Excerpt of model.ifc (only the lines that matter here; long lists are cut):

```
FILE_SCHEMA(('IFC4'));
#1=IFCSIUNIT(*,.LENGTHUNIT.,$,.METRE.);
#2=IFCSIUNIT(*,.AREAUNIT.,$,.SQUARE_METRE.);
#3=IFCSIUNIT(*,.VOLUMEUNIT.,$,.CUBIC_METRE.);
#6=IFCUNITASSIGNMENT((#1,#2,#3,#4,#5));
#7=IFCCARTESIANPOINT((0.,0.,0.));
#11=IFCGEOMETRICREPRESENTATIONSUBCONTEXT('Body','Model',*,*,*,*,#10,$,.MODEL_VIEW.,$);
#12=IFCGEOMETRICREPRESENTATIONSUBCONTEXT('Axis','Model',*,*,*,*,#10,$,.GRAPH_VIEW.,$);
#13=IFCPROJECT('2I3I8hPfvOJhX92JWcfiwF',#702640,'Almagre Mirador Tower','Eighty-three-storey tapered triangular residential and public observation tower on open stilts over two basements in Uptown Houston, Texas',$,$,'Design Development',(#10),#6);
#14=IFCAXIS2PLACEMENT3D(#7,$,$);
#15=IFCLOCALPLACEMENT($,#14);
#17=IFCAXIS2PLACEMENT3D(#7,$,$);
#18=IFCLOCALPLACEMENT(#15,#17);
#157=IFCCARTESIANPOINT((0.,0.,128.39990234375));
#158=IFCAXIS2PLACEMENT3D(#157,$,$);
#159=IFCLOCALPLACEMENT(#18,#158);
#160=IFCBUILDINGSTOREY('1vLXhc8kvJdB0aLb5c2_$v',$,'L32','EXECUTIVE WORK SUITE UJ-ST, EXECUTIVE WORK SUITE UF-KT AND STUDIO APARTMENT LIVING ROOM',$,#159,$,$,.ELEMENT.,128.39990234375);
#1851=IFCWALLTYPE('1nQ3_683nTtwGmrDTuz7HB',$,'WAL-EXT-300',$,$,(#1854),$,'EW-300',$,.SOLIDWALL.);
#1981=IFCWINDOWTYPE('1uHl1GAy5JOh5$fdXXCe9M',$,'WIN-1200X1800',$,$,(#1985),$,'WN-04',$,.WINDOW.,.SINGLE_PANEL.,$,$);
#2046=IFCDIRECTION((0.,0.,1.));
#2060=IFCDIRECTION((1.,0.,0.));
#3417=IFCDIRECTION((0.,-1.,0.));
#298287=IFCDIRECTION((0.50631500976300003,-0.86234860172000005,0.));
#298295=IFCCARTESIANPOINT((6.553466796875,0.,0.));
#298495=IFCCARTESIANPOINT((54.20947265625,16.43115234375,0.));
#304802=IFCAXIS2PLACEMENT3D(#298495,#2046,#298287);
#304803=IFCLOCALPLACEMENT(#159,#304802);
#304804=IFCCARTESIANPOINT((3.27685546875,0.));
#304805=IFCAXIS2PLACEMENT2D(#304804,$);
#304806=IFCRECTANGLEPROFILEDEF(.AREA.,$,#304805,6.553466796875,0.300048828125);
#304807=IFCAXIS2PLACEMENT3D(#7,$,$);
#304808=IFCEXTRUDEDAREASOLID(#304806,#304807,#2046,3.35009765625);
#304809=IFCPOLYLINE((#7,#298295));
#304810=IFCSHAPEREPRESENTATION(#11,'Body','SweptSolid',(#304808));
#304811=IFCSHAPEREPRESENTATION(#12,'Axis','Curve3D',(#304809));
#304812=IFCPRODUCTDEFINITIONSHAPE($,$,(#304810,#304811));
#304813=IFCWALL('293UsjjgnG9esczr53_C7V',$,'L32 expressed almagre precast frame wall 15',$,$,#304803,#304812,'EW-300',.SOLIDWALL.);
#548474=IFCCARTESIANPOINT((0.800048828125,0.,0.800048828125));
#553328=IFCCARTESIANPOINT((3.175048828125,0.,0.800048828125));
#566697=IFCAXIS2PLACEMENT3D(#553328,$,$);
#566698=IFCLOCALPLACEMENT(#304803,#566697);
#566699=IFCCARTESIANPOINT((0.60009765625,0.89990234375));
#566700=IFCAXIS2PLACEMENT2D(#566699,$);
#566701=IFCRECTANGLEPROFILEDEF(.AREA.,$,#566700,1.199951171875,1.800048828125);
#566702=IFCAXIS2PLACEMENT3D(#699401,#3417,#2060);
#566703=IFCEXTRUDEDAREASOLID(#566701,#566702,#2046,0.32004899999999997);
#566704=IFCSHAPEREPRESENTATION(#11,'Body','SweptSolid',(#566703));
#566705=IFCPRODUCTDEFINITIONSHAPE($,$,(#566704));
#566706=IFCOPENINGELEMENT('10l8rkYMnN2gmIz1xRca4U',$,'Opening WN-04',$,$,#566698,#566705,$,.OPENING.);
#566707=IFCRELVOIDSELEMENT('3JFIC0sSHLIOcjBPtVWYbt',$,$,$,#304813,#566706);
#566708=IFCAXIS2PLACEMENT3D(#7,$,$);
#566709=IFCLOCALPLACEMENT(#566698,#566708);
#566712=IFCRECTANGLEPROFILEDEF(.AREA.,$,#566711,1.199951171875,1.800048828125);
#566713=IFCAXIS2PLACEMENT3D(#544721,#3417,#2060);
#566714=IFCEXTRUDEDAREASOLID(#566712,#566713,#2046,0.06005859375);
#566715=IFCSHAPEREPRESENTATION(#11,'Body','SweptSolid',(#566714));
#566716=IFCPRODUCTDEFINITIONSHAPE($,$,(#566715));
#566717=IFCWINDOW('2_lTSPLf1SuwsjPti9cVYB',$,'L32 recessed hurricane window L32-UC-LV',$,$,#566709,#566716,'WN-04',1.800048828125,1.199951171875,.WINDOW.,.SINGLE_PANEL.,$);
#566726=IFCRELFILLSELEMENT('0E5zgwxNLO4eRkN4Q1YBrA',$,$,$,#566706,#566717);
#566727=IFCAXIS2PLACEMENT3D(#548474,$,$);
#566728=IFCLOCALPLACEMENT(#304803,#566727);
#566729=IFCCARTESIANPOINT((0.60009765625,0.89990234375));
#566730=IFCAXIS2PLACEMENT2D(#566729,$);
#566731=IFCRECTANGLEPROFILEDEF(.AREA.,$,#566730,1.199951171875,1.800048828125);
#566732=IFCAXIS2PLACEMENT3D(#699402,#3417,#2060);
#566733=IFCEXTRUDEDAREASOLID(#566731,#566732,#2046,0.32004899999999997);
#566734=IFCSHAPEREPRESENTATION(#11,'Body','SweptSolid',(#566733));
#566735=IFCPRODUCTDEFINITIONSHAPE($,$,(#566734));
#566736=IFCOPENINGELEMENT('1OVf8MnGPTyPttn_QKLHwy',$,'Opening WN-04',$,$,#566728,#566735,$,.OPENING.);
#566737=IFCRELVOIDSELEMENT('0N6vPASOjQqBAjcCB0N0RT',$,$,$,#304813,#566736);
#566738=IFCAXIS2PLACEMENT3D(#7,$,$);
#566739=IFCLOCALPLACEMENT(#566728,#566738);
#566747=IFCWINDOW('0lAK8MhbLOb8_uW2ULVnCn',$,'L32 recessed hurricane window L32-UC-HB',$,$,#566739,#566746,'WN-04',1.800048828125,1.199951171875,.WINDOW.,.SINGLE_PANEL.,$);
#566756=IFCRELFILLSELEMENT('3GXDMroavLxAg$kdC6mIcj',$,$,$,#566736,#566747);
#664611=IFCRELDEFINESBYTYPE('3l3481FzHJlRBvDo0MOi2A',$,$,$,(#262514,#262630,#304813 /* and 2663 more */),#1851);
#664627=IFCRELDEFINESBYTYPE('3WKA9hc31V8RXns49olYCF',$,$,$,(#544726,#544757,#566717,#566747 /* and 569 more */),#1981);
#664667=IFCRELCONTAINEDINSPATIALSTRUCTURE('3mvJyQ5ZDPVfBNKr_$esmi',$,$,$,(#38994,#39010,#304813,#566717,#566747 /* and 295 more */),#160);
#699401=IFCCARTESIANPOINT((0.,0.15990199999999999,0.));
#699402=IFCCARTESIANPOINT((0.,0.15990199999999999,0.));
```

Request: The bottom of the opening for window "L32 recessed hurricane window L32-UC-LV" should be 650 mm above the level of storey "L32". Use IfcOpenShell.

```python
import numpy as np
import ifcopenshell
import ifcopenshell.api.geometry
import ifcopenshell.geom
import ifcopenshell.util.element
import ifcopenshell.util.placement
import ifcopenshell.util.shape
import ifcopenshell.util.unit

model = ifcopenshell.open("model.ifc")
unit_scale = ifcopenshell.util.unit.calculate_unit_scale(model)

window = model.by_guid("2_lTSPLf1SuwsjPti9cVYB")
opening = window.FillsVoids[0].RelatingOpeningElement
storey = ifcopenshell.util.element.get_container(window, ifc_class="IfcBuildingStorey")
level = ifcopenshell.util.placement.get_local_placement(storey.ObjectPlacement)[2, 3]

# The opening's origin need not be at the sill, so measure its lowest point.
shape = ifcopenshell.geom.create_shape(ifcopenshell.geom.settings(), opening)
bottom = ifcopenshell.util.shape.get_shape_bottom_elevation(shape, shape.geometry) / unit_scale
dz = level + 0.65 / unit_scale - bottom

shift = np.array([0.0, 0.0, dz])
# The window is placed relative to its opening, so it follows when the opening moves.
matrix = ifcopenshell.util.placement.get_local_placement(opening.ObjectPlacement)
matrix[:3, 3] += shift
ifcopenshell.api.geometry.edit_object_placement(
    model, product=opening, matrix=matrix, is_si=False, should_transform_children=True
)

print(f"moved by {dz * unit_scale:+.3f} m")

model.write("model_v2.ifc")
```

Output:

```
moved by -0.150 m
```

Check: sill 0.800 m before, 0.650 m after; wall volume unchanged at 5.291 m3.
